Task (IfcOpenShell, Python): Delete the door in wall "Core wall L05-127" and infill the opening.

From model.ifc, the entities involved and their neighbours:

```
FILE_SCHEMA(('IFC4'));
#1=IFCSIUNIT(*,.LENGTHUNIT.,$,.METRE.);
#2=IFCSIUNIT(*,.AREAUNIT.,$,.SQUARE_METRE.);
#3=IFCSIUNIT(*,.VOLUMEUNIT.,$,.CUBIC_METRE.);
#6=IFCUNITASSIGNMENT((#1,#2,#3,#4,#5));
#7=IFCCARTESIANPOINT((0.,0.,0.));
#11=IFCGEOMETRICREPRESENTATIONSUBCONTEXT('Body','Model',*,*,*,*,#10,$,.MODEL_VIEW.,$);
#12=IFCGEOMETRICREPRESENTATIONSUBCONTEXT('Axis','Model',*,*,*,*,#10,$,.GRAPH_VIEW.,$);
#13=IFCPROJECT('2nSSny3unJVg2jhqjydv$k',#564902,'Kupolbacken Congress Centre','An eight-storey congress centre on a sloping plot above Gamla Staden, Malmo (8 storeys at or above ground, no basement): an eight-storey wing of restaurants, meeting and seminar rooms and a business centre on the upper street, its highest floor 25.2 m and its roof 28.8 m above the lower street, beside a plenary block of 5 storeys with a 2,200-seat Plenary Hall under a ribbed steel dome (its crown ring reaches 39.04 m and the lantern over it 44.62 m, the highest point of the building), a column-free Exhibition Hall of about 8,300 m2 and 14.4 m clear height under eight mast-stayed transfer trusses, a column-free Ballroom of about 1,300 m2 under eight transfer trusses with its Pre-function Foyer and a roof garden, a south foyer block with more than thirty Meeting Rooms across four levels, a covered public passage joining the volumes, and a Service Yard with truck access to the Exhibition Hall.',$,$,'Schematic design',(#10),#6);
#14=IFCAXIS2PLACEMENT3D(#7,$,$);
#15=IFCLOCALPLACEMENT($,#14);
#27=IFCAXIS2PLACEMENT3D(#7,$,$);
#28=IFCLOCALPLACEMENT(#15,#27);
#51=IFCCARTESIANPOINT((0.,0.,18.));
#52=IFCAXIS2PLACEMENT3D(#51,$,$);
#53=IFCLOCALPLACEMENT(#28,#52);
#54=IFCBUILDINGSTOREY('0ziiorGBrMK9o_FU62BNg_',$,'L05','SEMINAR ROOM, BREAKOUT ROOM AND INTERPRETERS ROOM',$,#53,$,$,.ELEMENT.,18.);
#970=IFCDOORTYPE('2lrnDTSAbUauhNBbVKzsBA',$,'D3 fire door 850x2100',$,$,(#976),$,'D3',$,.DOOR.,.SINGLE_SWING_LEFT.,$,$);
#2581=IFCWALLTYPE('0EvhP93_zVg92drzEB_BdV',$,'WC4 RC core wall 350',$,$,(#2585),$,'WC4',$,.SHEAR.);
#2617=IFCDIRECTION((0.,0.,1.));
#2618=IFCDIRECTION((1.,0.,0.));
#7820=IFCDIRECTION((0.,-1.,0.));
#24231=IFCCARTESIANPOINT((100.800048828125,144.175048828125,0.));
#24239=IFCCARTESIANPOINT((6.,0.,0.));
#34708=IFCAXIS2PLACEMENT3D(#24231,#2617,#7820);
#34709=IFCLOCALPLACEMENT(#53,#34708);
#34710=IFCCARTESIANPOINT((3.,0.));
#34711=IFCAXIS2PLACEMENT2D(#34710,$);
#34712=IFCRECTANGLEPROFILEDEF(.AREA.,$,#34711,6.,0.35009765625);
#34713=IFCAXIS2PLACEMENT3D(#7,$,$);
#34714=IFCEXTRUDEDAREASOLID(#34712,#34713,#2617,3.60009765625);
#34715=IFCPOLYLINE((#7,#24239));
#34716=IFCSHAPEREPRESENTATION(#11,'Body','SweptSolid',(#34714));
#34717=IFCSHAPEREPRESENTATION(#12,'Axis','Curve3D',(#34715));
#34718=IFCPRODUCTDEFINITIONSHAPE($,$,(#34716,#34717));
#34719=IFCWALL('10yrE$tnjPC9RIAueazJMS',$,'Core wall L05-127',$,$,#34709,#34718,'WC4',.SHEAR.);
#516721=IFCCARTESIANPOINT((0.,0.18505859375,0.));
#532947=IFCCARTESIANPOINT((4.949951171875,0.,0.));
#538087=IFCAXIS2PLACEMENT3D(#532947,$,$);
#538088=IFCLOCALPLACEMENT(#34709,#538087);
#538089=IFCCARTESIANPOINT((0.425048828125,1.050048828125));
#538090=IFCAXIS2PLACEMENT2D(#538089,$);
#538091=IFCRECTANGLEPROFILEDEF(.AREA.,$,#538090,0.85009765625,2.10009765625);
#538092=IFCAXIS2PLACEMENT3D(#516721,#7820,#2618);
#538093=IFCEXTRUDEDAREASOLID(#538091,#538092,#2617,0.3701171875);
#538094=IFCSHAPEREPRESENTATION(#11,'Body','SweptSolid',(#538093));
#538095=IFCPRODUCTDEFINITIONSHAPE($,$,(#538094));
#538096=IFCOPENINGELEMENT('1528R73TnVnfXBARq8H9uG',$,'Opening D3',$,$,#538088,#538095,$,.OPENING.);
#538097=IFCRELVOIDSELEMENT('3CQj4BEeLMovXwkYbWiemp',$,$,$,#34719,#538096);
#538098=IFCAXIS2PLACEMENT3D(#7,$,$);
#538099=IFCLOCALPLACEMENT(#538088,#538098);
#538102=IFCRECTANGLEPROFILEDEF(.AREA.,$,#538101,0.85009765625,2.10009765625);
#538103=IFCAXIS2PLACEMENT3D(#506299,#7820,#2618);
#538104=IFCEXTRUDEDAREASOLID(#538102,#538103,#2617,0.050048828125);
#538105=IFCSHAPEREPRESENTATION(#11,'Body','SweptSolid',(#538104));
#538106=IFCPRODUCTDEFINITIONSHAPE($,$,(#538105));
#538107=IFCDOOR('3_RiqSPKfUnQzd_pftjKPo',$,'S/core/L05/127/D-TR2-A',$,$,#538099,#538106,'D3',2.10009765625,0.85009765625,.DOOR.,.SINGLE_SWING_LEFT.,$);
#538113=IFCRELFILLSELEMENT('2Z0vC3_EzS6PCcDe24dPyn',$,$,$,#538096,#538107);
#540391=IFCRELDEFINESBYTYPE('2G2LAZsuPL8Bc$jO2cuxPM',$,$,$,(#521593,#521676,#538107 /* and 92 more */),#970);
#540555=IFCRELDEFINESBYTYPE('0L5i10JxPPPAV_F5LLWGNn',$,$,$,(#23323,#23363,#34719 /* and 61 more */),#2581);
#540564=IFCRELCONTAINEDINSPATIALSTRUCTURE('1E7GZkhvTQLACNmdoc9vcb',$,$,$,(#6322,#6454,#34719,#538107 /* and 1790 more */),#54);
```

```python
import ifcopenshell
import ifcopenshell.api.feature
import ifcopenshell.api.root
import ifcopenshell.geom
import ifcopenshell.util.shape

model = ifcopenshell.open("model.ifc")
settings = ifcopenshell.geom.settings()


def volume(element):
    """Net volume in cubic metres, openings subtracted."""
    shape = ifcopenshell.geom.create_shape(settings, element)
    return ifcopenshell.util.shape.get_volume(shape.geometry)


door = model.by_guid("3_RiqSPKfUnQzd_pftjKPo")
opening = door.FillsVoids[0].RelatingOpeningElement
wall = opening.VoidsElements[0].RelatingBuildingElement
before = volume(wall)

ifcopenshell.api.root.remove_product(model, product=door)
ifcopenshell.api.feature.remove_feature(model, feature=opening)

after = volume(wall)

print(f"wall volume {before:.3f} -> {after:.3f} m3")

model.write("model_edited.ifc")
```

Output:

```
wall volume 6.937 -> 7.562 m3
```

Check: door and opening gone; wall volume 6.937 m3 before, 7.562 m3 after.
